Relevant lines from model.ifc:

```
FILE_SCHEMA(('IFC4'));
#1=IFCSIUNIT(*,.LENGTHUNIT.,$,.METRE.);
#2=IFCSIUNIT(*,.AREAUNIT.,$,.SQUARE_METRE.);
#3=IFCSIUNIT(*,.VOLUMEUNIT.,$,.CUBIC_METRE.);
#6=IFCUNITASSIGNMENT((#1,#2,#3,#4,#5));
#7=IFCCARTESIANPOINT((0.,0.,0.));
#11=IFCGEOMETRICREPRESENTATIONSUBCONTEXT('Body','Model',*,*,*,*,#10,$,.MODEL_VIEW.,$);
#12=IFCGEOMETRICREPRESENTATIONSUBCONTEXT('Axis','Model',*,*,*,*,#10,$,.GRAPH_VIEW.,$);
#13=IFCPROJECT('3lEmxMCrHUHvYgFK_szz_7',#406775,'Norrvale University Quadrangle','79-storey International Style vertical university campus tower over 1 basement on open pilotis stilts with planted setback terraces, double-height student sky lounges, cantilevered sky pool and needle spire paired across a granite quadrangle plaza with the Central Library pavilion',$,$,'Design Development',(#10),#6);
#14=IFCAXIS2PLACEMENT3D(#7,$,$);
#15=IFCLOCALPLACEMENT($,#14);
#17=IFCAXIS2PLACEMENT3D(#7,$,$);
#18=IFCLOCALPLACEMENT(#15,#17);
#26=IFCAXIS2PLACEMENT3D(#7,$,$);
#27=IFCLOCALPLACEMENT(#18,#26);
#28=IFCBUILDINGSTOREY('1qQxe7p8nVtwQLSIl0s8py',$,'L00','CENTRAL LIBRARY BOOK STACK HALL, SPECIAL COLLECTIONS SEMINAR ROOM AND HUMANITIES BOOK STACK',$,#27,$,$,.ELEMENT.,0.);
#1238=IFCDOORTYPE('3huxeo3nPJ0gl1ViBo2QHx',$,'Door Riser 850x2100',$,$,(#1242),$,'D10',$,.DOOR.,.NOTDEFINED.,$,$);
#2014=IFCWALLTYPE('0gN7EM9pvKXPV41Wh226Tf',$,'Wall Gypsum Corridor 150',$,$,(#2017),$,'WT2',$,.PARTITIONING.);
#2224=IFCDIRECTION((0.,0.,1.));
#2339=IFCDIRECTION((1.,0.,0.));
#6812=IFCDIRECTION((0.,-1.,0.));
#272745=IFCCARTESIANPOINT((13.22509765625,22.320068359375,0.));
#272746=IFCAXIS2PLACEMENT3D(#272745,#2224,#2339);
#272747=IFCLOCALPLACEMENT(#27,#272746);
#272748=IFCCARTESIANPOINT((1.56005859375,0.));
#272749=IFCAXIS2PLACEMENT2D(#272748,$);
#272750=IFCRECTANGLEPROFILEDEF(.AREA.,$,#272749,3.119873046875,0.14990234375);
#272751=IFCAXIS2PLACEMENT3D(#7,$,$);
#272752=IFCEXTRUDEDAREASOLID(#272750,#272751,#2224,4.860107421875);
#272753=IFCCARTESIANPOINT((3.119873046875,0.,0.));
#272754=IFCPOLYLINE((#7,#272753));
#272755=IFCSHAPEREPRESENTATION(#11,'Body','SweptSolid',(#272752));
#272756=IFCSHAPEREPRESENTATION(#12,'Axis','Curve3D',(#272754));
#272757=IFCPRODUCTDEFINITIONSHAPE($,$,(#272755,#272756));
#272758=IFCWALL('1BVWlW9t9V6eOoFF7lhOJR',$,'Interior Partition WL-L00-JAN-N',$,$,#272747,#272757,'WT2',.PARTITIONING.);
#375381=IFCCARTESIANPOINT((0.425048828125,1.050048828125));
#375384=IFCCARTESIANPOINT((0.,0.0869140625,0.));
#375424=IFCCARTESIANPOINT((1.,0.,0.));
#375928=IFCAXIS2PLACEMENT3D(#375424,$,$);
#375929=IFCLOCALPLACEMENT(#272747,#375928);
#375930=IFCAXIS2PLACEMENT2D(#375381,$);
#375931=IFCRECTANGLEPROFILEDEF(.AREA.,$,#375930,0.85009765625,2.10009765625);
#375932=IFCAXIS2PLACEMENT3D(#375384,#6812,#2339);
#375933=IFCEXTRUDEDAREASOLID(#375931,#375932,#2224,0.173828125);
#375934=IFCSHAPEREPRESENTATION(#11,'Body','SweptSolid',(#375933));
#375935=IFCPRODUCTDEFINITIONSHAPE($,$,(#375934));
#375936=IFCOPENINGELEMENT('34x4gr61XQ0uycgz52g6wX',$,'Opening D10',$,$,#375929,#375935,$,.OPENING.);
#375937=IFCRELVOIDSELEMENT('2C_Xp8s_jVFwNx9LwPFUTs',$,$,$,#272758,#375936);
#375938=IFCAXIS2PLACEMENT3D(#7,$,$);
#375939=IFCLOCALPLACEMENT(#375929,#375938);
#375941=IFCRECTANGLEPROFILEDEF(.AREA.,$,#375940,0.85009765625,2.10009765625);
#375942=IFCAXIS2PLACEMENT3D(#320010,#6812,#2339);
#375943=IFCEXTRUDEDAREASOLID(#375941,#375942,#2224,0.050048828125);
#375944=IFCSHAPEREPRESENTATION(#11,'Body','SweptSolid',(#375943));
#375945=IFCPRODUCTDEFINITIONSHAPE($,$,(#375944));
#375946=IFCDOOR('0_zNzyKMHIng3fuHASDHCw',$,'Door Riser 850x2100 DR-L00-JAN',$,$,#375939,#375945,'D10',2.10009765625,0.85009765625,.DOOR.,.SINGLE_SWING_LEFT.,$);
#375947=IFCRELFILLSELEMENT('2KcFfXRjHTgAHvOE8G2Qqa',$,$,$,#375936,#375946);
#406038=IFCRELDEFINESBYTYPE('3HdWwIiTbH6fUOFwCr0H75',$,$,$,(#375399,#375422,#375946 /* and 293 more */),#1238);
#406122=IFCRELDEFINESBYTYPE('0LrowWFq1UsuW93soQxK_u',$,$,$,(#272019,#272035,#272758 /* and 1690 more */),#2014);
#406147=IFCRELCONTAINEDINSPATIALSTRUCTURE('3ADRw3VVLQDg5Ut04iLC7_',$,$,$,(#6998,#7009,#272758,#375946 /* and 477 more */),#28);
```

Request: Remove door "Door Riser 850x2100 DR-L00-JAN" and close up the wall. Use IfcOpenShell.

```python
import ifcopenshell
import ifcopenshell.api.feature
import ifcopenshell.api.root
import ifcopenshell.geom
import ifcopenshell.util.shape

model = ifcopenshell.open("model.ifc")
settings = ifcopenshell.geom.settings()


def volume(element):
    """Net volume in cubic metres, openings subtracted."""
    shape = ifcopenshell.geom.create_shape(settings, element)
    return ifcopenshell.util.shape.get_volume(shape.geometry)


door = model.by_id(375946)
opening = door.FillsVoids[0].RelatingOpeningElement
wall = opening.VoidsElements[0].RelatingBuildingElement
before = volume(wall)

ifcopenshell.api.root.remove_product(model, product=door)
ifcopenshell.api.feature.remove_feature(model, feature=opening)

after = volume(wall)

print(f"wall volume {before:.3f} -> {after:.3f} m3")

model.write("model_v2.ifc")
```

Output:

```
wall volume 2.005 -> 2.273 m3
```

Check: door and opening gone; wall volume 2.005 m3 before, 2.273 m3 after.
